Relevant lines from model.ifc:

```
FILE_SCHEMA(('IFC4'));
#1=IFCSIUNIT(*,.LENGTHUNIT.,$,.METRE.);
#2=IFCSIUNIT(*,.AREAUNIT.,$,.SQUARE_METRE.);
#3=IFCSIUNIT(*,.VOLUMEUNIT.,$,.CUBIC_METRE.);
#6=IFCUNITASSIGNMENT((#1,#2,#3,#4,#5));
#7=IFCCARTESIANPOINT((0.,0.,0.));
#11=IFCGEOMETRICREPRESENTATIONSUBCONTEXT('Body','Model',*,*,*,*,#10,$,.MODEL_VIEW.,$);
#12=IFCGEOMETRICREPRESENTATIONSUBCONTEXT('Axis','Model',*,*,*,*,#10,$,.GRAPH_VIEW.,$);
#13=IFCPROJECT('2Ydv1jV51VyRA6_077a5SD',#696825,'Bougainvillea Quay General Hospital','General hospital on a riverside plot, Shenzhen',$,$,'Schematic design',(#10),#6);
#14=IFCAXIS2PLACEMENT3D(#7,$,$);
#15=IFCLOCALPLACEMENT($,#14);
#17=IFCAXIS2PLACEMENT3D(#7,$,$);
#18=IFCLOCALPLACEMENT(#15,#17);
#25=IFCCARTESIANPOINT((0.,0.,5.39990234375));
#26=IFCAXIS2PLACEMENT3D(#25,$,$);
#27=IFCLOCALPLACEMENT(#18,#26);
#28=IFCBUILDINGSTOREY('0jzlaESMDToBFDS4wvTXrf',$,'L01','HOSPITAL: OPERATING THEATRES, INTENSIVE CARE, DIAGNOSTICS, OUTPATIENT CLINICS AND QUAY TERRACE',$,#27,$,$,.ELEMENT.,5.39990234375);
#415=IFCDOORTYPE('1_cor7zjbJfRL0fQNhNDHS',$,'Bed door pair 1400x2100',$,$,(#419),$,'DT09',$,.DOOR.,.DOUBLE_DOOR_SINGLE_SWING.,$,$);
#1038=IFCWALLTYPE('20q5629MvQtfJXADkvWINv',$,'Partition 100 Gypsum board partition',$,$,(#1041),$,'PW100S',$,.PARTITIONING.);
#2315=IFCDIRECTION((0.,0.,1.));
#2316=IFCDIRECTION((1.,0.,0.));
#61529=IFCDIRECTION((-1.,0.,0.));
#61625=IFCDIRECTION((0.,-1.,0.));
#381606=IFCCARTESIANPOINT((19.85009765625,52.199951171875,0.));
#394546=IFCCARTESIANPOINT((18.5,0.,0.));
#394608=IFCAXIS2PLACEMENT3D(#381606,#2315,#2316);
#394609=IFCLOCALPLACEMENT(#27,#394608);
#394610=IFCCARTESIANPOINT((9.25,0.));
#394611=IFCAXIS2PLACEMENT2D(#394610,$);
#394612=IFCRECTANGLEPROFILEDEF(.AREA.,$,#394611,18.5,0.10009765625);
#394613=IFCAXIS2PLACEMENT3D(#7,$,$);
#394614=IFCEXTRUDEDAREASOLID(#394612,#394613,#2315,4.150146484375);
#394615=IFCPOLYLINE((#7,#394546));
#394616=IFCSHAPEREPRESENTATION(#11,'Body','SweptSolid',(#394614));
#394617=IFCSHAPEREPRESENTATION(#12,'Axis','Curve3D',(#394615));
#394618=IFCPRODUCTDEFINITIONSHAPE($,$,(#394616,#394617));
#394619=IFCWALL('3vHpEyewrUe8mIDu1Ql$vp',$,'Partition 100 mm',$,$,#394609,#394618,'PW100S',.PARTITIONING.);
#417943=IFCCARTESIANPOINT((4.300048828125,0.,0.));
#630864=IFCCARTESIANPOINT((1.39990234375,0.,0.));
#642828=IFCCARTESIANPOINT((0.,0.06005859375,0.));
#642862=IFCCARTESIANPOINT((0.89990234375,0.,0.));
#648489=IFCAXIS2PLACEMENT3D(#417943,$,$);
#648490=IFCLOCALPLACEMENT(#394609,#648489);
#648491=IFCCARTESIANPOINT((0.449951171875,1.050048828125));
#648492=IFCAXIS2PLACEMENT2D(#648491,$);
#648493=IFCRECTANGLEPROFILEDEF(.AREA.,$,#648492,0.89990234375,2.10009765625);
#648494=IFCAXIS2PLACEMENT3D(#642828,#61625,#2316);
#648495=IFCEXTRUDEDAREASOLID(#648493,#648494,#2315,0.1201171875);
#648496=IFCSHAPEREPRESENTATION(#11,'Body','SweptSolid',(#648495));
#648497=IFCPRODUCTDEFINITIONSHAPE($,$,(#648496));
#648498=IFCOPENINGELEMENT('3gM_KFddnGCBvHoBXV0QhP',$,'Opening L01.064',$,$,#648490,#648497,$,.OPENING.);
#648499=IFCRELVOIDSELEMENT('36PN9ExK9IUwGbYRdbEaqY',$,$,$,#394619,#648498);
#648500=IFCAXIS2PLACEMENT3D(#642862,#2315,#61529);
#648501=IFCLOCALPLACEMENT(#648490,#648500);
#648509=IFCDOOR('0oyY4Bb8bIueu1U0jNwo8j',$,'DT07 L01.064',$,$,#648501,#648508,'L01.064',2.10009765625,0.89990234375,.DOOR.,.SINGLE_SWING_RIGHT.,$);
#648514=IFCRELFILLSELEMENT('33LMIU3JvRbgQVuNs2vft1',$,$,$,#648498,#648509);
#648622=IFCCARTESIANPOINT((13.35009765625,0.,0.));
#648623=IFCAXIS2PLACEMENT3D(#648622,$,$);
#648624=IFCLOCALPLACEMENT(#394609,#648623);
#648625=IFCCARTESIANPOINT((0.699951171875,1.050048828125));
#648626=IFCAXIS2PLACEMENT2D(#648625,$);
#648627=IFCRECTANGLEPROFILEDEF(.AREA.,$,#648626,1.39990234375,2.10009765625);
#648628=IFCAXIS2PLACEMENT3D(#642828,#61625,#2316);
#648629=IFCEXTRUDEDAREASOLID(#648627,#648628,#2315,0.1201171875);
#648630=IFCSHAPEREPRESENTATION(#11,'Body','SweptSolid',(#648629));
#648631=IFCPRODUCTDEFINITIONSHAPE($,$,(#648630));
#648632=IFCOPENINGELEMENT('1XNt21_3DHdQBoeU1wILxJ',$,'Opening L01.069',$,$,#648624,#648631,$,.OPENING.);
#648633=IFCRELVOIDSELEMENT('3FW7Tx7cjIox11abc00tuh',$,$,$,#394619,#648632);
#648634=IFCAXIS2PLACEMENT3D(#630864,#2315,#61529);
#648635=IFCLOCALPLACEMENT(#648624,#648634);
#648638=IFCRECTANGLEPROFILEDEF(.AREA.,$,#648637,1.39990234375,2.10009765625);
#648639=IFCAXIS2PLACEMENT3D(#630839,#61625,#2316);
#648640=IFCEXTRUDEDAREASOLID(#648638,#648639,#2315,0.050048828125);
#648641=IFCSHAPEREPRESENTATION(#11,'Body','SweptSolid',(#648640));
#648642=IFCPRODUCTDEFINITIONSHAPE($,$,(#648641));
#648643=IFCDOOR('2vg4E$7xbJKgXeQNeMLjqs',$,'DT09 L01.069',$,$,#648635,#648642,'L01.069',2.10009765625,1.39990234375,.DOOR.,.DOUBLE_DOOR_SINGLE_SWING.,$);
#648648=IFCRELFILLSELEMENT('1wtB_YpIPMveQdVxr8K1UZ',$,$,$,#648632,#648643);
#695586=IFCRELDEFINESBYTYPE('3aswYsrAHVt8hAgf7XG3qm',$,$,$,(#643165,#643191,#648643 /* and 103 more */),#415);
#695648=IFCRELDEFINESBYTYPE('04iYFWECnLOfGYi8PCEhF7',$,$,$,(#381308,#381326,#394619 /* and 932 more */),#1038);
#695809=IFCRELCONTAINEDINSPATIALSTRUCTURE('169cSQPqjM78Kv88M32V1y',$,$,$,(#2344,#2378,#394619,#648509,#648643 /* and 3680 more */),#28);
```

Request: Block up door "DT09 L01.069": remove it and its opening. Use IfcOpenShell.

```python
import ifcopenshell
import ifcopenshell.api.feature
import ifcopenshell.api.root
import ifcopenshell.geom
import ifcopenshell.util.shape

model = ifcopenshell.open("model.ifc")
settings = ifcopenshell.geom.settings()


def volume(element):
    """Net volume in cubic metres, openings subtracted."""
    shape = ifcopenshell.geom.create_shape(settings, element)
    return ifcopenshell.util.shape.get_volume(shape.geometry)


door = model.by_id(648643)
opening = door.FillsVoids[0].RelatingOpeningElement
wall = opening.VoidsElements[0].RelatingBuildingElement
before = volume(wall)

ifcopenshell.api.root.remove_product(model, product=door)
ifcopenshell.api.feature.remove_feature(model, feature=opening)

after = volume(wall)

print(f"wall volume {before:.3f} -> {after:.3f} m3")

model.write("model_edited.ifc")
```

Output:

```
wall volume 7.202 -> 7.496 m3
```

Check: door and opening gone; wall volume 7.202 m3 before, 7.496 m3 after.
